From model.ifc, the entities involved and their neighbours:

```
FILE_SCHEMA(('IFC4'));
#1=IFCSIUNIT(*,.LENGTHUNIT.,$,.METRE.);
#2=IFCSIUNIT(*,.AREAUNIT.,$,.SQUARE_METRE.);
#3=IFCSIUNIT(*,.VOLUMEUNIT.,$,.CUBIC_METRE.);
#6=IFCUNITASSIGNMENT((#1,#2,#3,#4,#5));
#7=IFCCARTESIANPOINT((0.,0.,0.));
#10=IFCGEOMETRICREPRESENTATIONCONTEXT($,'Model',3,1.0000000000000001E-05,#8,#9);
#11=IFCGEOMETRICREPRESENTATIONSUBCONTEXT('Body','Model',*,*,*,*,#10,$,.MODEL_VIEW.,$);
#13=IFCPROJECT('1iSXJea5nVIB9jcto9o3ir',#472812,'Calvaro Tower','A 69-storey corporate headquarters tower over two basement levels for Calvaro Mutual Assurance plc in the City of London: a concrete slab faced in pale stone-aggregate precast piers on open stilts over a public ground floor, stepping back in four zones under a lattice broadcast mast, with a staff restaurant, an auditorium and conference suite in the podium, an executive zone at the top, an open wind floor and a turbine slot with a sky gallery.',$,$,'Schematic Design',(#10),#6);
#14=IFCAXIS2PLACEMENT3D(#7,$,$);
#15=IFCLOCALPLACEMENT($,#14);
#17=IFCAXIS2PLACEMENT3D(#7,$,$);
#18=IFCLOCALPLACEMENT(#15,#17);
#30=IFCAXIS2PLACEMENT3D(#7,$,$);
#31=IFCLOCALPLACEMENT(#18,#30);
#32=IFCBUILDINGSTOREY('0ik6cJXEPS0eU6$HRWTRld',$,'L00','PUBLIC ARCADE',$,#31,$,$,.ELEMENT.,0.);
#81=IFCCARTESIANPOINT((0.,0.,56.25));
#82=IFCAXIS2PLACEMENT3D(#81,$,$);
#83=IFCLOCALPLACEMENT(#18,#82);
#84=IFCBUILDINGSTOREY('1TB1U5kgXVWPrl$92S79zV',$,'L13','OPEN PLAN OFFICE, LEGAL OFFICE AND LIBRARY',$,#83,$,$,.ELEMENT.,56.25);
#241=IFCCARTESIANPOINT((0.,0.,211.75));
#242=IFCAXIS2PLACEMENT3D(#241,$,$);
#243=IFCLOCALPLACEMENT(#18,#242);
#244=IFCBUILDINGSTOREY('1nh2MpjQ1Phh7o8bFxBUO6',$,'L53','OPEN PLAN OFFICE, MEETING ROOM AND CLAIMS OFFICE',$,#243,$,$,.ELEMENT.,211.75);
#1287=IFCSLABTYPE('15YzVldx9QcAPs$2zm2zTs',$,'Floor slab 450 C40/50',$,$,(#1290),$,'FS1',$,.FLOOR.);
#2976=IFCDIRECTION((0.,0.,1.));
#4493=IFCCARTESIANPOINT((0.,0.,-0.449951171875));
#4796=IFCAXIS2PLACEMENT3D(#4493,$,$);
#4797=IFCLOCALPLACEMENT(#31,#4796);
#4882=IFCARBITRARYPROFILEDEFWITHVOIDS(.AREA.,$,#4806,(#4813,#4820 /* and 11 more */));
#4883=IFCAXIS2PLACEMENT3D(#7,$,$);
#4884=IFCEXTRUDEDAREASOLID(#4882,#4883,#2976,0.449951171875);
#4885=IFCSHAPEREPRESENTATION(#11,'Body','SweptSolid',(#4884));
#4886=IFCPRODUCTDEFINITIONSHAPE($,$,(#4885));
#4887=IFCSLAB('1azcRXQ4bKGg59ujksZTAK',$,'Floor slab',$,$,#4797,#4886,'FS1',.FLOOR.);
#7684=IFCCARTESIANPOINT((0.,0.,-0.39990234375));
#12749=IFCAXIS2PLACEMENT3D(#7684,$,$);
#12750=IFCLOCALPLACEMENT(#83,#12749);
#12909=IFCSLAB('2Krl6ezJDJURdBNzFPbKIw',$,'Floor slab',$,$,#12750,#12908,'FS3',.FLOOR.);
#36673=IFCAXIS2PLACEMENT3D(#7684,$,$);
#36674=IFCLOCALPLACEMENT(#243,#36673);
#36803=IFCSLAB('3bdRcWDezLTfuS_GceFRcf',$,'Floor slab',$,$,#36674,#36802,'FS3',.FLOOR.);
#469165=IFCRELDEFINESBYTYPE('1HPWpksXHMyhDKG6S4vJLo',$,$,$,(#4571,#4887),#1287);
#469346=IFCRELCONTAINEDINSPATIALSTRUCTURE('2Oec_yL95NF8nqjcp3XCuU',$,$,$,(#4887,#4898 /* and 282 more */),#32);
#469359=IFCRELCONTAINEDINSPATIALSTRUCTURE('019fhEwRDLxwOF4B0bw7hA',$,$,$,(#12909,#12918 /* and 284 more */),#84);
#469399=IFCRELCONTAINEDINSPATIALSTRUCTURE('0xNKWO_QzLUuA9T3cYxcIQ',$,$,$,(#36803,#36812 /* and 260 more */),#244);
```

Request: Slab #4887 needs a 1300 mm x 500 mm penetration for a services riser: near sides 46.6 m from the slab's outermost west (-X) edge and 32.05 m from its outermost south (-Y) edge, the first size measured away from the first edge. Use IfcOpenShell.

```python
import numpy as np
import ifcopenshell
import ifcopenshell.api.feature
import ifcopenshell.api.geometry
import ifcopenshell.api.root
import ifcopenshell.geom
import ifcopenshell.util.placement
import ifcopenshell.util.representation
import ifcopenshell.util.shape
import ifcopenshell.util.unit

model = ifcopenshell.open("model.ifc")
unit_scale = ifcopenshell.util.unit.calculate_unit_scale(model)
settings = ifcopenshell.geom.settings()


def volume(element):
    """Net volume in cubic metres, openings subtracted."""
    shape = ifcopenshell.geom.create_shape(settings, element)
    return ifcopenshell.util.shape.get_volume(shape.geometry)


slab = model.by_guid("1azcRXQ4bKGg59ujksZTAK")
before = volume(slab)

# Extent in the slab's own axes, in metres. The edges named are its -X and -Y sides.
slab_shape = ifcopenshell.geom.create_shape(settings, slab)
vertices = ifcopenshell.util.shape.get_vertices(slab_shape.geometry)
x_min, y_min, bottom = vertices.min(axis=0)
top = vertices[:, 2].max()

opening = ifcopenshell.api.root.create_entity(model, ifc_class="IfcOpeningElement", name="Services riser opening", predefined_type="OPENING")
context = ifcopenshell.util.representation.get_context(model, "Model", "Body", "MODEL_VIEW")
width, depth = 1.3, 0.5
outline = [(0.0, 0.0), (width, 0.0), (width, depth), (0.0, depth), (0.0, 0.0)]
# Overshoot both faces by 50 mm so the cut is clean.
shape = ifcopenshell.api.geometry.add_slab_representation(
    model, context=context, depth=top - bottom + 0.1, polyline=outline
)
ifcopenshell.api.geometry.assign_representation(model, product=opening, representation=shape)

matrix = ifcopenshell.util.placement.get_local_placement(slab.ObjectPlacement)
matrix[:, 3] = matrix @ np.append(np.array([x_min + 46.6, y_min + 32.05, bottom - 0.05]) / unit_scale, 1.0)
ifcopenshell.api.geometry.edit_object_placement(model, product=opening, matrix=matrix, is_si=False)
ifcopenshell.api.feature.add_feature(model, feature=opening, element=slab)

after = volume(slab)

print(f"slab volume {before:.3f} -> {after:.3f} m3")

model.write("model_edited.ifc")
```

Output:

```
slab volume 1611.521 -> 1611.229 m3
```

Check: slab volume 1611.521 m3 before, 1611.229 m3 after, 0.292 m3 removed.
